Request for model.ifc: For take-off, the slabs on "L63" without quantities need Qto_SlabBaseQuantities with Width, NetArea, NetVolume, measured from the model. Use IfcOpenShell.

First a look at what the model holds.

```python
import ifcopenshell
import ifcopenshell.util.element
import ifcopenshell.util.unit

model = ifcopenshell.open("model.ifc")
print(model.schema)
for unit_type in ("LENGTHUNIT", "AREAUNIT", "VOLUMEUNIT"):
    print(unit_type, ifcopenshell.util.unit.calculate_unit_scale(model, unit_type))
storey = next(s for s in model.by_type("IfcBuildingStorey") if s.Name == "L63")
slabs = [e for e in ifcopenshell.util.element.get_decomposition(storey) if e.is_a("IfcSlab")]
for e in sorted(slabs, key=lambda e: e.id()):
    print(e.id(), e.is_a(), e.Name, list(ifcopenshell.util.element.get_psets(e, qtos_only=True)), sep=" | ")
```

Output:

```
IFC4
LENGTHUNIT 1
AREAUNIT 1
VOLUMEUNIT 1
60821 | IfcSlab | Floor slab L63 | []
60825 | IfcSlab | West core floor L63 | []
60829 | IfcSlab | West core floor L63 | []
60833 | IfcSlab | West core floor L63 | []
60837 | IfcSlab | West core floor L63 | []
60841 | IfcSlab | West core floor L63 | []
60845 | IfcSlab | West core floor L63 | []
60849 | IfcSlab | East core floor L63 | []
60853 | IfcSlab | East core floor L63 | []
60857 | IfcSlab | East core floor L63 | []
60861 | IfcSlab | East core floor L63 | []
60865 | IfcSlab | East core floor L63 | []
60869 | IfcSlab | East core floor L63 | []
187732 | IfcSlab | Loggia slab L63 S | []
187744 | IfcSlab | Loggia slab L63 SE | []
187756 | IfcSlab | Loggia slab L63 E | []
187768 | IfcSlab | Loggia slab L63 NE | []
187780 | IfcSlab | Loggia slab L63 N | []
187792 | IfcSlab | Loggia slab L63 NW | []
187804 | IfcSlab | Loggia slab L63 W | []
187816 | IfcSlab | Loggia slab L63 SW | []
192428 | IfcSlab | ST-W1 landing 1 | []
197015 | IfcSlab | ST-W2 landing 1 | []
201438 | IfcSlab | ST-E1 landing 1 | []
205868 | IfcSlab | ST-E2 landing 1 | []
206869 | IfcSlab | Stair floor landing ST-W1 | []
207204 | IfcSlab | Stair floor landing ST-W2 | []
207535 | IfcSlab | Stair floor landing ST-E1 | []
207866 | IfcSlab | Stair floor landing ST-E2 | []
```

```python
import ifcopenshell
import ifcopenshell.api.pset
import ifcopenshell.geom
import ifcopenshell.util.element
import ifcopenshell.util.shape
import ifcopenshell.util.unit

model = ifcopenshell.open("model.ifc")
unit_scale = ifcopenshell.util.unit.calculate_unit_scale(model)
area_scale = ifcopenshell.util.unit.calculate_unit_scale(model, "AREAUNIT")
volume_scale = ifcopenshell.util.unit.calculate_unit_scale(model, "VOLUMEUNIT")
settings = ifcopenshell.geom.settings()

storey = next(s for s in model.by_type("IfcBuildingStorey") if s.Name == "L63")
slabs = [e for e in ifcopenshell.util.element.get_decomposition(storey) if e.is_a("IfcSlab")]

for e in sorted(slabs, key=lambda e: e.id()):
    if ifcopenshell.util.element.get_psets(e, qtos_only=True, should_inherit=False):
        continue
    # Geometry comes back in metres, in the element's own axes.
    shape = ifcopenshell.geom.create_shape(settings, e)
    values = {
        "Width": ifcopenshell.util.shape.get_z(shape.geometry) / unit_scale,
        "NetArea": ifcopenshell.util.shape.get_footprint_area(shape.geometry) / area_scale,
        "NetVolume": ifcopenshell.util.shape.get_volume(shape.geometry) / volume_scale,
    }
    qto = ifcopenshell.api.pset.add_qto(model, product=e, name="Qto_SlabBaseQuantities")
    ifcopenshell.api.pset.edit_qto(model, qto=qto, properties=values)
    print(e.id(), {k: round(v, 3) for k, v in values.items()})

model.write("model_v2.ifc")
```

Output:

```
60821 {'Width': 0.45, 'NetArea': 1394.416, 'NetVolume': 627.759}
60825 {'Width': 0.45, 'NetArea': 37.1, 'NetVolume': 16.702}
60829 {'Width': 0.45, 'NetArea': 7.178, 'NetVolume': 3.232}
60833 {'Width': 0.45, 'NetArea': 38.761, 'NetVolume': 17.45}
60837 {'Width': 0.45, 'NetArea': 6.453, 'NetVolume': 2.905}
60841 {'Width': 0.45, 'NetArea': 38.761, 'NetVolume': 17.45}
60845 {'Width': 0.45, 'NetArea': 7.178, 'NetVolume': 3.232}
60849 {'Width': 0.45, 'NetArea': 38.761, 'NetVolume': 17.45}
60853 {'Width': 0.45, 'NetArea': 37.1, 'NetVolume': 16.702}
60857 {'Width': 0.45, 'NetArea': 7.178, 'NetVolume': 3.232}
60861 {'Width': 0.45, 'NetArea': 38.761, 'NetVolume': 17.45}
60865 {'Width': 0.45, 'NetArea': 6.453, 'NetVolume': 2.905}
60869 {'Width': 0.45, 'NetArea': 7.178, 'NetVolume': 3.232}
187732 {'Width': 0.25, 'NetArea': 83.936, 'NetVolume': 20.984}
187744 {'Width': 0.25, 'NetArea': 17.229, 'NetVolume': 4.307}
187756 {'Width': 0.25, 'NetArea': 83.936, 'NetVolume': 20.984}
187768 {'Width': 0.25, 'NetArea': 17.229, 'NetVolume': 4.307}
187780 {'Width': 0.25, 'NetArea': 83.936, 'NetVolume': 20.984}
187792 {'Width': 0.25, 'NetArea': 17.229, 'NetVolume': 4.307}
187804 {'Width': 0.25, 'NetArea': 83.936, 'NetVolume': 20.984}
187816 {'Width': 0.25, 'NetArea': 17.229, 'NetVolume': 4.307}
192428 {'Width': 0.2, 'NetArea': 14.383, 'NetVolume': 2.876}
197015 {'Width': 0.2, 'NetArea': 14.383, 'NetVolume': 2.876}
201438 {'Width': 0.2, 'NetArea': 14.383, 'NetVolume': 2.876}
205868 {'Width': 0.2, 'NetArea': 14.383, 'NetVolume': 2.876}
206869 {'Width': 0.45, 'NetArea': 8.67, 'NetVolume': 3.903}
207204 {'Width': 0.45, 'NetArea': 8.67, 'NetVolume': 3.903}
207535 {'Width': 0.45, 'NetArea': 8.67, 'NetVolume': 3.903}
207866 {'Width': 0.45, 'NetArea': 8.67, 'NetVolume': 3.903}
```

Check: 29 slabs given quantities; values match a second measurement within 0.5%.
